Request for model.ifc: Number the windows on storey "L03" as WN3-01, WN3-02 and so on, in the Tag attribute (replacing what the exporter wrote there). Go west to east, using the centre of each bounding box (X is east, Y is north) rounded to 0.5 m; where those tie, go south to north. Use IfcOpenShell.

First a look at what the model holds.

```python
import ifcopenshell
import ifcopenshell.util.element
import ifcopenshell.util.placement

model = ifcopenshell.open("model.ifc")
print(model.schema)
storey = next(s for s in model.by_type("IfcBuildingStorey") if s.Name == "L03")
windows = [e for e in ifcopenshell.util.element.get_decomposition(storey) if e.is_a("IfcWindow")]
for e in sorted(windows, key=lambda e: e.id()):
    origin = ifcopenshell.util.placement.get_local_placement(e.ObjectPlacement)[:3, 3]
    print(e.id(), e.Tag, e.Name, origin.round(2) + 0.0, sep=" | ")
```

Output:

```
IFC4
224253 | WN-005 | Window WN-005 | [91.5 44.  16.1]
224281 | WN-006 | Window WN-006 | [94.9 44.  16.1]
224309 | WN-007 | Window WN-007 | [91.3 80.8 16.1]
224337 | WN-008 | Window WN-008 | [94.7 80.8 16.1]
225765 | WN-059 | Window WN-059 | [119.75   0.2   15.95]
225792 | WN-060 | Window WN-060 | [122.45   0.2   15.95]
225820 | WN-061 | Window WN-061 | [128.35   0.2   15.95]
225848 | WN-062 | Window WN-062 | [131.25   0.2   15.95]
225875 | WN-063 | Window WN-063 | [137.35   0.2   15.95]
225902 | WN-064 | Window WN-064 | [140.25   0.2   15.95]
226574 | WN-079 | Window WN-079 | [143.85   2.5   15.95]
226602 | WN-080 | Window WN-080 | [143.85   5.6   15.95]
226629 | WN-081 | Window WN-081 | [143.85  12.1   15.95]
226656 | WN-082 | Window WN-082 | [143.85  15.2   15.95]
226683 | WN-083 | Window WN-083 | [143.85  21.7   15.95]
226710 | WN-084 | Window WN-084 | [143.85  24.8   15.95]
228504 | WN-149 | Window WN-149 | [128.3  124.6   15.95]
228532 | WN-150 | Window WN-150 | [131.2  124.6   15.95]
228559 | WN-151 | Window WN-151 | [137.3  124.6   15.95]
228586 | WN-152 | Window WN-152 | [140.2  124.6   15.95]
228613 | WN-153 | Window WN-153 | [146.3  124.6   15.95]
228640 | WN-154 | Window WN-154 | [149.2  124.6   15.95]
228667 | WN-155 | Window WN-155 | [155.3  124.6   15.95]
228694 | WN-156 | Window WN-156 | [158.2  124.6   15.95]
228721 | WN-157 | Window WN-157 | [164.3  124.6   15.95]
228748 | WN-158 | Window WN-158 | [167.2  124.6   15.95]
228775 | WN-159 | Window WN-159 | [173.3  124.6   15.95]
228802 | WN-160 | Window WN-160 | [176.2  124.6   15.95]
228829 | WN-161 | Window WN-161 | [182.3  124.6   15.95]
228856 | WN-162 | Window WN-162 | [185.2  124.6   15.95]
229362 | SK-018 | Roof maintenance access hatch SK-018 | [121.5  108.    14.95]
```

```python
import ifcopenshell
import ifcopenshell.geom
import ifcopenshell.util.element
import ifcopenshell.util.shape

model = ifcopenshell.open("model.ifc")
settings = ifcopenshell.geom.settings()
settings.set("use-world-coords", True)


def centre(element):
    shape = ifcopenshell.geom.create_shape(settings, element)
    return ifcopenshell.util.shape.get_bbox_centroid(shape.geometry)


storey = next(s for s in model.by_type("IfcBuildingStorey") if s.Name == "L03")
windows = [e for e in ifcopenshell.util.element.get_decomposition(storey) if e.is_a("IfcWindow")]

# Insertion points can sit at a corner or the storey origin, so sort by the geometry (in metres).
centres = {e: centre(e) for e in windows}
windows.sort(key=lambda e: (round(centres[e][0] / 0.5), centres[e][1]))

for i, e in enumerate(windows, start=1):
    number = f"WN3-{i:02d}"
    e.Tag = number
    print(e.id(), number)

model.write("model-out.ifc")
```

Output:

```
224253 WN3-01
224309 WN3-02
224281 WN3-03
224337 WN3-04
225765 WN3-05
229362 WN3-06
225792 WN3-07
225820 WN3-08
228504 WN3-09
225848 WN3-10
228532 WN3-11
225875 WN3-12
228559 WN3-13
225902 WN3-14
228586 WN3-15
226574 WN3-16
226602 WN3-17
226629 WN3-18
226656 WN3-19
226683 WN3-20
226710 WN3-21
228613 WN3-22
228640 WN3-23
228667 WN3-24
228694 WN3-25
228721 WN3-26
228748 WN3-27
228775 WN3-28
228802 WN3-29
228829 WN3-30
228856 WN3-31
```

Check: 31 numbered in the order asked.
